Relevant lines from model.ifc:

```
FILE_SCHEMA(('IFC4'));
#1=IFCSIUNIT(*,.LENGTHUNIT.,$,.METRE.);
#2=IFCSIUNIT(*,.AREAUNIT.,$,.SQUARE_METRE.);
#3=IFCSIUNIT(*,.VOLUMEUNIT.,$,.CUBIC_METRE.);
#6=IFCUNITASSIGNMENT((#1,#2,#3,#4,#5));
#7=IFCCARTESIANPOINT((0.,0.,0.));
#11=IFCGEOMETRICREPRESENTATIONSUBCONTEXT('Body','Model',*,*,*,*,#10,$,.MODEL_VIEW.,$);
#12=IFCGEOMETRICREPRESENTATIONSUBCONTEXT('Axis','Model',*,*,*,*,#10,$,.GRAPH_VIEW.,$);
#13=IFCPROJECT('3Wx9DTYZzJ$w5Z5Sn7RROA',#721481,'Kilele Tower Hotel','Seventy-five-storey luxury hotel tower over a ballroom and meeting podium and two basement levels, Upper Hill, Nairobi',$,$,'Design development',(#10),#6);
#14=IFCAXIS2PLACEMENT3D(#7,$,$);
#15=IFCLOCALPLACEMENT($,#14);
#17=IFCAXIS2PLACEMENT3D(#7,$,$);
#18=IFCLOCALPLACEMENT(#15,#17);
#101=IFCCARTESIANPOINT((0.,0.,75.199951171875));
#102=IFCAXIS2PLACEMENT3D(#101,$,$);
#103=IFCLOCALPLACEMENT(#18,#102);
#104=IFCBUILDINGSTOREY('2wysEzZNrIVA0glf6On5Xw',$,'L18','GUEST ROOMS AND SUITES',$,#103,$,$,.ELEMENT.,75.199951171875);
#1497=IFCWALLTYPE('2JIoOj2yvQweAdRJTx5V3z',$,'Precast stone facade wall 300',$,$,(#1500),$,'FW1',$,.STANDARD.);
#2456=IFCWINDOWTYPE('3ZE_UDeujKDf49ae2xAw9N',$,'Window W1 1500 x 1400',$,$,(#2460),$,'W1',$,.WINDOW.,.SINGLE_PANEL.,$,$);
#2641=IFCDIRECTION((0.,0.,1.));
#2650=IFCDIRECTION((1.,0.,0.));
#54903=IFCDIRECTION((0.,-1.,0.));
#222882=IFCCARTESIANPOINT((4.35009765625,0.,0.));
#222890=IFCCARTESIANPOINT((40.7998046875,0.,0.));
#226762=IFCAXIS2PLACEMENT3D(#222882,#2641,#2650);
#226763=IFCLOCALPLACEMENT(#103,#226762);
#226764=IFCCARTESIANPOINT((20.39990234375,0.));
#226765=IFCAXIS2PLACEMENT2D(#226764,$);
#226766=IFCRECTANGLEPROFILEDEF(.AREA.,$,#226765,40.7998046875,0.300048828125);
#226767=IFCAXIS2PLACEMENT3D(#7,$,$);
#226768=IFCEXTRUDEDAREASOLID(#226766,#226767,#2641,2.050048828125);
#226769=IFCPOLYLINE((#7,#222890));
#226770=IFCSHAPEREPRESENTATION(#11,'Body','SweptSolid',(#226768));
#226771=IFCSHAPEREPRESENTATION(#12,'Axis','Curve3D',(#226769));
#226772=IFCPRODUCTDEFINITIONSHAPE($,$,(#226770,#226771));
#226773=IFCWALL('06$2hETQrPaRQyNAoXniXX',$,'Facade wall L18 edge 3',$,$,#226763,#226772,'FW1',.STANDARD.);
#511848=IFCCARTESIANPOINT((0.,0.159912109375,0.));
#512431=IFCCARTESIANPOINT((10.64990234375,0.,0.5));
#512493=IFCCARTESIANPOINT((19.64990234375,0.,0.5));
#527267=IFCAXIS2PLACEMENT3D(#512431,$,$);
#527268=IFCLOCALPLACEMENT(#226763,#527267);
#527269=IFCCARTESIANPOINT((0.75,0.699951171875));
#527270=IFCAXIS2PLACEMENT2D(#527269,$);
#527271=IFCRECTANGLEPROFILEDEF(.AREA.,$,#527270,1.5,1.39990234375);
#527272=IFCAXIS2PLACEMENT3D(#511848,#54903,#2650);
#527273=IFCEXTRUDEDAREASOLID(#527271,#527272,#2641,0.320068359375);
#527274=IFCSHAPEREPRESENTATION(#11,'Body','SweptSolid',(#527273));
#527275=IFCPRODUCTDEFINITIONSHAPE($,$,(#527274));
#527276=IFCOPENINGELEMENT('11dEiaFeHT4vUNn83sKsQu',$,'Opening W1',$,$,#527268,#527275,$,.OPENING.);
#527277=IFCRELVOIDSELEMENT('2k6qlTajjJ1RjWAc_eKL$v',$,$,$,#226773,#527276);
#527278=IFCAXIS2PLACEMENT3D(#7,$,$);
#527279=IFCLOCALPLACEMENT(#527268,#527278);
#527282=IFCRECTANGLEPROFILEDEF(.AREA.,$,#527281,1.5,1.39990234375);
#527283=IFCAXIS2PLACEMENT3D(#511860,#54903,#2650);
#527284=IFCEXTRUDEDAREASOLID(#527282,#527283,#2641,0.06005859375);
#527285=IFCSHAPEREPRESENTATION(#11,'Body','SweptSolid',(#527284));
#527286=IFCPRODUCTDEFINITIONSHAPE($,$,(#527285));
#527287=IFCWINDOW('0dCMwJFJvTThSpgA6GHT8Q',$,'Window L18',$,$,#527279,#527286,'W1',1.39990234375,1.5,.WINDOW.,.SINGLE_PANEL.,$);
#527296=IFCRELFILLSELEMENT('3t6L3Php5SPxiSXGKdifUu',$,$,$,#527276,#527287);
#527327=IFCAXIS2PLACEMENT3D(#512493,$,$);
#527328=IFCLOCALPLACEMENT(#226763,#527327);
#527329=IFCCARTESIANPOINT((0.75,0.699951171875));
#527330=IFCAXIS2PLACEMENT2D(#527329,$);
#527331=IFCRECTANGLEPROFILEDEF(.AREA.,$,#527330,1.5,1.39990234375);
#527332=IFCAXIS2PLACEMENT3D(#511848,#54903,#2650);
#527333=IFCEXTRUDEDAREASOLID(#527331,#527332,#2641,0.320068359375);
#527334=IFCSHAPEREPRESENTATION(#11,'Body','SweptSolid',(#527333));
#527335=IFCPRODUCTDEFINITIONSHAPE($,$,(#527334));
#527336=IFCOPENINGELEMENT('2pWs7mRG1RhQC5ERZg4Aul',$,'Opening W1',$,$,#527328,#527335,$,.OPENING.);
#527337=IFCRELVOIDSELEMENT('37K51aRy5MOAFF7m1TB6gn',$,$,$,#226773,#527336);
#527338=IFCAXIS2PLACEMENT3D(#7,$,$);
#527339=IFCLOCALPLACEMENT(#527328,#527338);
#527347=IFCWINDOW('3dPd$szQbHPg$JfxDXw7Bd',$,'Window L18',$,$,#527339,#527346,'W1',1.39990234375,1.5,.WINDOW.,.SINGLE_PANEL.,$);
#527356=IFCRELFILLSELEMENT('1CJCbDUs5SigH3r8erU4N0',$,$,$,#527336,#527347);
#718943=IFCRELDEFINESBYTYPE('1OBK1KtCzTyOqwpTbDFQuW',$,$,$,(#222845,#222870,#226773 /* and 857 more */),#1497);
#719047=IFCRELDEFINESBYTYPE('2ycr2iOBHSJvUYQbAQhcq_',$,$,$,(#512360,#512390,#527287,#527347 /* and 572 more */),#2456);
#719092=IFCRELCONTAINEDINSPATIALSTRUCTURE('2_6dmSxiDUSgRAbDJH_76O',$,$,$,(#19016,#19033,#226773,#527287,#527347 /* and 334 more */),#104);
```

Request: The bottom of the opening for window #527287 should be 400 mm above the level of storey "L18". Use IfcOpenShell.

```python
import numpy as np
import ifcopenshell
import ifcopenshell.api.geometry
import ifcopenshell.geom
import ifcopenshell.util.element
import ifcopenshell.util.placement
import ifcopenshell.util.shape
import ifcopenshell.util.unit

model = ifcopenshell.open("model.ifc")
unit_scale = ifcopenshell.util.unit.calculate_unit_scale(model)

window = model.by_id(527287)
opening = window.FillsVoids[0].RelatingOpeningElement
storey = ifcopenshell.util.element.get_container(window, ifc_class="IfcBuildingStorey")
level = ifcopenshell.util.placement.get_local_placement(storey.ObjectPlacement)[2, 3]

# The opening's origin need not be at the sill, so measure its lowest point.
shape = ifcopenshell.geom.create_shape(ifcopenshell.geom.settings(), opening)
bottom = ifcopenshell.util.shape.get_shape_bottom_elevation(shape, shape.geometry) / unit_scale
dz = level + 0.4 - bottom

shift = np.array([0.0, 0.0, dz])
# The window is placed relative to its opening, so it follows when the opening moves.
matrix = ifcopenshell.util.placement.get_local_placement(opening.ObjectPlacement)
matrix[:3, 3] += shift
ifcopenshell.api.geometry.edit_object_placement(
    model, product=opening, matrix=matrix, is_si=False, should_transform_children=True
)

print(f"moved by {dz * unit_scale:+.3f} m")

model.write("model_v2.ifc")
```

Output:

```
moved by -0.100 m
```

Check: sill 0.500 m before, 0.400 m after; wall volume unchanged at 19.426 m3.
